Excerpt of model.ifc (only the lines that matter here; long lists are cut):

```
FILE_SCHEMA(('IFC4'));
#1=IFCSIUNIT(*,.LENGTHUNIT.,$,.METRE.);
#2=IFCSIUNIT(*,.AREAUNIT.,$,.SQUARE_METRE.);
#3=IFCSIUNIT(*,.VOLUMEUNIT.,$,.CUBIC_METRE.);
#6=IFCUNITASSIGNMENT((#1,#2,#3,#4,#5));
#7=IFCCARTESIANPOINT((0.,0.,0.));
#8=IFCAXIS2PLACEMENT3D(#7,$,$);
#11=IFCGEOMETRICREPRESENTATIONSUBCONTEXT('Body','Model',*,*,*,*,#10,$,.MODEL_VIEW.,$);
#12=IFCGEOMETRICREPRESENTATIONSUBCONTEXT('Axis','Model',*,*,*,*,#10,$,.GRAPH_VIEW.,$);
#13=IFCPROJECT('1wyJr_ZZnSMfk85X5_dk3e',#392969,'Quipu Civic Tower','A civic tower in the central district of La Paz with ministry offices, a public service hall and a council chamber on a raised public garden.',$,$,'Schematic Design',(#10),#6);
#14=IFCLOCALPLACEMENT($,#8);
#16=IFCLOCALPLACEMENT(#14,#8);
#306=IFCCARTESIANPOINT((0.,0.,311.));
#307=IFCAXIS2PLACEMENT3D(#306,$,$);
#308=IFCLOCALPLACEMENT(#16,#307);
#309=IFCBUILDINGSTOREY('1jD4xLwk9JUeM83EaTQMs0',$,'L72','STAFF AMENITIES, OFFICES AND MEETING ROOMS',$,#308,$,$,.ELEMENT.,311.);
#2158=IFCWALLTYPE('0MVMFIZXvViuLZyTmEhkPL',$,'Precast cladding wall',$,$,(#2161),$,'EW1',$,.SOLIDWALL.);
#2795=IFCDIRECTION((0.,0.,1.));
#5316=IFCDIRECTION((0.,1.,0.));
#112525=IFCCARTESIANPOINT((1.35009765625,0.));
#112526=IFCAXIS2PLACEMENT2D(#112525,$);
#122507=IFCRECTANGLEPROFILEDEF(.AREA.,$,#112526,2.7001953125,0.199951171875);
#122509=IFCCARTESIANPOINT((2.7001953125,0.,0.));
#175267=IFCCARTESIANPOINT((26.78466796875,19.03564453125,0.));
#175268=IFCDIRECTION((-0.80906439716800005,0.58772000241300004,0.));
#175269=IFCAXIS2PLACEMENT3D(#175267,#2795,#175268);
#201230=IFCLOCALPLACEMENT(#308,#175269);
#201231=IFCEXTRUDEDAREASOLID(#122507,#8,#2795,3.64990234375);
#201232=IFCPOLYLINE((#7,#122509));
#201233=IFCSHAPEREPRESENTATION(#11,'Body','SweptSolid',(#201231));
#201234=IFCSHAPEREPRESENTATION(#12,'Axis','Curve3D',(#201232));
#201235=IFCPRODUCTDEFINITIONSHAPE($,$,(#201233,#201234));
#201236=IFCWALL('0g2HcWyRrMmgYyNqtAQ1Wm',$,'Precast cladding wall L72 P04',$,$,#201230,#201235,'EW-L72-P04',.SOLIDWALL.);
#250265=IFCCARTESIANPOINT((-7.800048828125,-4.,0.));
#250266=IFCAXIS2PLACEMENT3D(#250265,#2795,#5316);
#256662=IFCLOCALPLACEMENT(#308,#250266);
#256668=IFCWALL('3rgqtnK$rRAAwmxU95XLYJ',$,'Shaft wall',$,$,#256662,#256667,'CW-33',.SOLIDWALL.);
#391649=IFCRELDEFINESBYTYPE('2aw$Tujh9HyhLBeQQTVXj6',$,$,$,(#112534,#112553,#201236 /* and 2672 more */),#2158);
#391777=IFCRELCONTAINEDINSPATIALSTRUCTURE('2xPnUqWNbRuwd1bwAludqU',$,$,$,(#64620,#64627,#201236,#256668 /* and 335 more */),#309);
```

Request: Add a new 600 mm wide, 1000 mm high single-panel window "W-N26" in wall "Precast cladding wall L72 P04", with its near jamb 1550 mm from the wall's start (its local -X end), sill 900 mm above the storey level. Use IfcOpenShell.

```python
import numpy as np
import ifcopenshell
import ifcopenshell.api.feature
import ifcopenshell.api.geometry
import ifcopenshell.api.root
import ifcopenshell.api.spatial
import ifcopenshell.geom
import ifcopenshell.util.element
import ifcopenshell.util.placement
import ifcopenshell.util.representation
import ifcopenshell.util.shape
import ifcopenshell.util.unit

model = ifcopenshell.open("model.ifc")
unit_scale = ifcopenshell.util.unit.calculate_unit_scale(model)
settings = ifcopenshell.geom.settings()


def volume(element):
    """Net volume in cubic metres, openings subtracted."""
    shape = ifcopenshell.geom.create_shape(settings, element)
    return ifcopenshell.util.shape.get_volume(shape.geometry)


wall = model.by_id(201236)
storey = ifcopenshell.util.element.get_container(wall, ifc_class="IfcBuildingStorey")
context = ifcopenshell.util.representation.get_context(model, "Model", "Body", "MODEL_VIEW")
before = volume(wall)

width, height, from_end, sill = 0.6, 1, 1.55, 0.9  # metres

# The wall runs along its own X axis, and the end named is its -X end.
wall_shape = ifcopenshell.geom.create_shape(settings, wall)
x, y, z = ifcopenshell.util.shape.get_vertices(wall_shape.geometry).T
start = x.min() + from_end
face, thickness = float(y.min()), float(y.max() - y.min())
wall_matrix = ifcopenshell.util.placement.get_local_placement(wall.ObjectPlacement)
level = ifcopenshell.util.placement.get_local_placement(storey.ObjectPlacement)[2, 3]


def in_wall(x, y):
    """Placement at x, y metres in the wall's axes, at sill height."""
    matrix = wall_matrix.copy()
    matrix[:, 3] = wall_matrix @ np.array([x / unit_scale, y / unit_scale, 0.0, 1.0])
    matrix[2, 3] = level + sill / unit_scale
    return matrix


# Opening: a box that overshoots both wall faces by 50 mm.
opening = ifcopenshell.api.root.create_entity(model, ifc_class="IfcOpeningElement", predefined_type="OPENING")
box = ifcopenshell.api.geometry.add_wall_representation(
    model, context=context, length=width, height=height, thickness=thickness + 0.1
)
ifcopenshell.api.geometry.assign_representation(model, product=opening, representation=box)
ifcopenshell.api.geometry.edit_object_placement(model, product=opening, matrix=in_wall(start, face - 0.05), is_si=False)
ifcopenshell.api.feature.add_feature(model, feature=opening, element=wall)

window = ifcopenshell.api.root.create_entity(model, ifc_class="IfcWindow", name="W-N26", predefined_type="WINDOW")
window.OverallWidth, window.OverallHeight = width / unit_scale, height / unit_scale
window.PartitioningType = "SINGLE_PANEL"
body = ifcopenshell.api.geometry.add_window_representation(
    model,
    context=context,
    overall_width=window.OverallWidth,
    overall_height=window.OverallHeight,
    partition_type="SINGLE_PANEL",
)
ifcopenshell.api.geometry.assign_representation(model, product=window, representation=body)
ifcopenshell.api.spatial.assign_container(model, products=[window], relating_structure=storey)
ifcopenshell.api.feature.add_filling(model, opening=opening, element=window)

# Centre the window in the wall's thickness.
ifcopenshell.api.geometry.edit_object_placement(model, product=window, matrix=in_wall(start, face), is_si=False)
window_shape = ifcopenshell.geom.create_shape(settings, window)
depth = ifcopenshell.util.shape.get_vertices(window_shape.geometry)[:, 1]
offset = face + thickness / 2 - (depth.min() + depth.max()) / 2
ifcopenshell.api.geometry.edit_object_placement(model, product=window, matrix=in_wall(start, offset), is_si=False)

after = volume(wall)

print(f"wall volume {before:.3f} -> {after:.3f} m3")

model.write("model-out.ifc")
```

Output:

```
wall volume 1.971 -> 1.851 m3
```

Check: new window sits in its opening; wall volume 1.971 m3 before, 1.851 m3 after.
